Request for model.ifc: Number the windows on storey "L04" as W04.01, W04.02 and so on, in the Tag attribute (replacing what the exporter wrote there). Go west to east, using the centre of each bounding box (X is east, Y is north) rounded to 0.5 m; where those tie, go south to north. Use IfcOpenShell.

First a look at what the model holds.

```python
import ifcopenshell
import ifcopenshell.util.element
import ifcopenshell.util.placement

model = ifcopenshell.open("model.ifc")
print(model.schema)
storey = next(s for s in model.by_type("IfcBuildingStorey") if s.Name == "L04")
windows = [e for e in ifcopenshell.util.element.get_decomposition(storey) if e.is_a("IfcWindow")]
for e in sorted(windows, key=lambda e: e.id()):
    origin = ifcopenshell.util.placement.get_local_placement(e.ObjectPlacement)[:3, 3]
    print(e.id(), e.Tag, e.Name, origin.round(2) + 0.0, sep=" | ")
```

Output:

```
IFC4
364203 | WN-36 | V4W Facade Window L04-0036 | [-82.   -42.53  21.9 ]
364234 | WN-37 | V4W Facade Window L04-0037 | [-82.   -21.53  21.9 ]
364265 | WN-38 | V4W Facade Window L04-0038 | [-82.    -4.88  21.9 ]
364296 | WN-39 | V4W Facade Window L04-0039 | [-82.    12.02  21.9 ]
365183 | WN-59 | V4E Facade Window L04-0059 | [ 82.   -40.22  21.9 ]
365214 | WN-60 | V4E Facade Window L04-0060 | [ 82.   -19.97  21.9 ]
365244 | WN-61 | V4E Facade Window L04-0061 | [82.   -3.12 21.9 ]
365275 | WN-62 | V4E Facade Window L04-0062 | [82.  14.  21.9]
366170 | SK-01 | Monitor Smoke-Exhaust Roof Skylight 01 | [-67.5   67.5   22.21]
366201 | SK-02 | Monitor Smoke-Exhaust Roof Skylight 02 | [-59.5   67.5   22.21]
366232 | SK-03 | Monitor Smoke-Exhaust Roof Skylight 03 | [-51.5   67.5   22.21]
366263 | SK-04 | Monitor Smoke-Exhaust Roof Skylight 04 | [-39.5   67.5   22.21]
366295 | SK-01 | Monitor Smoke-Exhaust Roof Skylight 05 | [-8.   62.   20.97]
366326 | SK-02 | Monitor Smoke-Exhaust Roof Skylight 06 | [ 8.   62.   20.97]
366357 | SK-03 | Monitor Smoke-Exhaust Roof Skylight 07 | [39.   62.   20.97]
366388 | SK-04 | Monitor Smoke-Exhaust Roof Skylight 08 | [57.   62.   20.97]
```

```python
import ifcopenshell
import ifcopenshell.geom
import ifcopenshell.util.element
import ifcopenshell.util.shape

model = ifcopenshell.open("model.ifc")
settings = ifcopenshell.geom.settings()
settings.set("use-world-coords", True)


def centre(element):
    shape = ifcopenshell.geom.create_shape(settings, element)
    return ifcopenshell.util.shape.get_bbox_centroid(shape.geometry)


storey = next(s for s in model.by_type("IfcBuildingStorey") if s.Name == "L04")
windows = [e for e in ifcopenshell.util.element.get_decomposition(storey) if e.is_a("IfcWindow")]

# Insertion points can sit at a corner or the storey origin, so sort by the geometry (in metres).
centres = {e: centre(e) for e in windows}
windows.sort(key=lambda e: (round(centres[e][0] / 0.5), centres[e][1]))

for i, e in enumerate(windows, start=1):
    number = f"W04.{i:02d}"
    e.Tag = number
    print(e.id(), number)

model.write("model-out.ifc")
```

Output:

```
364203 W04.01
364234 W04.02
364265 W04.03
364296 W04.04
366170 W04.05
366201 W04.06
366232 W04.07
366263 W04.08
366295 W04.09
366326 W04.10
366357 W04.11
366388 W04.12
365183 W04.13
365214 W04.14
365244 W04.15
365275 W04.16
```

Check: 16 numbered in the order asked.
